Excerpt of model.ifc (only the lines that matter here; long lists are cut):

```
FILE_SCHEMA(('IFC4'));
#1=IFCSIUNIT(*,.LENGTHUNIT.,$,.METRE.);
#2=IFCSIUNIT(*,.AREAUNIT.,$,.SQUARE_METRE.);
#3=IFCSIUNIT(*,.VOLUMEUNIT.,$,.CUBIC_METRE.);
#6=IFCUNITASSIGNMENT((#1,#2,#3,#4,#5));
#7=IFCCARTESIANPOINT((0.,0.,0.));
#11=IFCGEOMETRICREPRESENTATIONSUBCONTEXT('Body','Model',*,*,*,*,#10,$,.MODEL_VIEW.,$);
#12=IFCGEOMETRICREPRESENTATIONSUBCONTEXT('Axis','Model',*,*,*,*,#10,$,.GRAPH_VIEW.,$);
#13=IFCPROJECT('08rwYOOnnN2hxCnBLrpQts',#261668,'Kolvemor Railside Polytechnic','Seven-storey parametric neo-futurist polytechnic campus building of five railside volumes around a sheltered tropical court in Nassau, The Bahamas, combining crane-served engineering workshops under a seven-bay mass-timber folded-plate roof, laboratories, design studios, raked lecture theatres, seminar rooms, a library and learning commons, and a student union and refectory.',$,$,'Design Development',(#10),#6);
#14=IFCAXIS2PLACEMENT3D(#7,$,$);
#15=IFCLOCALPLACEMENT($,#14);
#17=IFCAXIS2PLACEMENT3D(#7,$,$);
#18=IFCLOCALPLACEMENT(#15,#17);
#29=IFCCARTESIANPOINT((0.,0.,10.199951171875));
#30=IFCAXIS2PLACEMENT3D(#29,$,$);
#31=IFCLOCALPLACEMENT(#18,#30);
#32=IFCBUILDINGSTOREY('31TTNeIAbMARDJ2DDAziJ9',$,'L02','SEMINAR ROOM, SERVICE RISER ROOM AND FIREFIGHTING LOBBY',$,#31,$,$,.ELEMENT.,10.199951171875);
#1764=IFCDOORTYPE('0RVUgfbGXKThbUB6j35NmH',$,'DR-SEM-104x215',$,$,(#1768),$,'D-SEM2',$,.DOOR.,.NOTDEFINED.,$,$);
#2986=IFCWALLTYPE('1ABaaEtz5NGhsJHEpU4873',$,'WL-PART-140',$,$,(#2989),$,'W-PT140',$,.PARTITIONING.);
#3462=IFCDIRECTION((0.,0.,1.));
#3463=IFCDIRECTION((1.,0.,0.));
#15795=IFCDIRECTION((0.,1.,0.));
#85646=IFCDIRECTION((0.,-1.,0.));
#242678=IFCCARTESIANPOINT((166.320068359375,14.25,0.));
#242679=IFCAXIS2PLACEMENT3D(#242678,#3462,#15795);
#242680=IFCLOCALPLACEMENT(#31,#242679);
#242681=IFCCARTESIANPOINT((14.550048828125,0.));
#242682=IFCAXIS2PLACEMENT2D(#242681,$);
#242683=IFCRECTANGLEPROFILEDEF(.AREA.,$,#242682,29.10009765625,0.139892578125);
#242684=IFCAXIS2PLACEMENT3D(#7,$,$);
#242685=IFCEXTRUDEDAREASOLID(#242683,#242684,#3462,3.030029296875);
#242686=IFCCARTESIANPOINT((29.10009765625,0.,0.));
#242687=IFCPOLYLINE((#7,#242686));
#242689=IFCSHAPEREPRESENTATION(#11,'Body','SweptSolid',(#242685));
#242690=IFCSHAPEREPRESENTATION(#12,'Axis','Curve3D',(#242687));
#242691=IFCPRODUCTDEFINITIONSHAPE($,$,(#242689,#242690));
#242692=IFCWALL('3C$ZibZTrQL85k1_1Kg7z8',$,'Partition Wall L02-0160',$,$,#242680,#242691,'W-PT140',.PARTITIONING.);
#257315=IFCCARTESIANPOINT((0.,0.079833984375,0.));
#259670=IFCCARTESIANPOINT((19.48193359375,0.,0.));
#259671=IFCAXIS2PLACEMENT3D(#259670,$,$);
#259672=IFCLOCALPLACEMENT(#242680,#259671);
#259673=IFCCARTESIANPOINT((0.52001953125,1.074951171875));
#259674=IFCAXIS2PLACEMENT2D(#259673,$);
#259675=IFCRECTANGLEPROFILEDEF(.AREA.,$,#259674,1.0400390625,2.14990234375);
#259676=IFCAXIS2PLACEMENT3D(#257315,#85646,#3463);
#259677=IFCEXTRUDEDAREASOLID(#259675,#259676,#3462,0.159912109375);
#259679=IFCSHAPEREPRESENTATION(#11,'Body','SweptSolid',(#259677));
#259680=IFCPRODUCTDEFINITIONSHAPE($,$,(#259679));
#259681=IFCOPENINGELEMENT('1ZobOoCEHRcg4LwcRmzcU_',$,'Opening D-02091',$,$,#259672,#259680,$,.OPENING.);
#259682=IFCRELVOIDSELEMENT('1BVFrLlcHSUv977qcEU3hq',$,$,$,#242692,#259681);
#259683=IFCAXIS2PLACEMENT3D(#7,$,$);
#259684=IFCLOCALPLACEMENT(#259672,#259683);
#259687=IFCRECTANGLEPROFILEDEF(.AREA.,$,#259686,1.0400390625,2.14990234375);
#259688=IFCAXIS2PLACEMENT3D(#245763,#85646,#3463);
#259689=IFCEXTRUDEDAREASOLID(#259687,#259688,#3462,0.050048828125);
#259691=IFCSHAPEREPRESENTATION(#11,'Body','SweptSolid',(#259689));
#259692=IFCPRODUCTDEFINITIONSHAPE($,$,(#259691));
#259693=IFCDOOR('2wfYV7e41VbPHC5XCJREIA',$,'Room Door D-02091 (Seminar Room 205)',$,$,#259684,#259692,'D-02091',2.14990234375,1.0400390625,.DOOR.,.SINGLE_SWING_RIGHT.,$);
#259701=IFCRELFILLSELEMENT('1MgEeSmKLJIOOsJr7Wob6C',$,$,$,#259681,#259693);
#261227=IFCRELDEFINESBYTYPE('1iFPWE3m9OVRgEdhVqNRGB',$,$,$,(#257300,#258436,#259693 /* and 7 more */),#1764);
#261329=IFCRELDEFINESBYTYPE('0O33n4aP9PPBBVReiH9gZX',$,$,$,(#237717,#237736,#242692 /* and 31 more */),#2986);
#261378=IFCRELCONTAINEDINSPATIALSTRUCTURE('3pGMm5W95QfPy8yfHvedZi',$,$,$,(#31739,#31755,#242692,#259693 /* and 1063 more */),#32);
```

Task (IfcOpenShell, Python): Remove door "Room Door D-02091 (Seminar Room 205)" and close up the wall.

```python
import ifcopenshell
import ifcopenshell.api.feature
import ifcopenshell.api.root
import ifcopenshell.geom
import ifcopenshell.util.shape

model = ifcopenshell.open("model.ifc")
settings = ifcopenshell.geom.settings()


def volume(element):
    """Net volume in cubic metres, openings subtracted."""
    shape = ifcopenshell.geom.create_shape(settings, element)
    return ifcopenshell.util.shape.get_volume(shape.geometry)


door = model.by_id(259693)
opening = door.FillsVoids[0].RelatingOpeningElement
wall = opening.VoidsElements[0].RelatingBuildingElement
before = volume(wall)

ifcopenshell.api.root.remove_product(model, product=door)
ifcopenshell.api.feature.remove_feature(model, feature=opening)

after = volume(wall)

print(f"wall volume {before:.3f} -> {after:.3f} m3")

model.write("model_v2.ifc")
```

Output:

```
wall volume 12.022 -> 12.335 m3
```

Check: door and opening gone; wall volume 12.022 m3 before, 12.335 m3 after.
